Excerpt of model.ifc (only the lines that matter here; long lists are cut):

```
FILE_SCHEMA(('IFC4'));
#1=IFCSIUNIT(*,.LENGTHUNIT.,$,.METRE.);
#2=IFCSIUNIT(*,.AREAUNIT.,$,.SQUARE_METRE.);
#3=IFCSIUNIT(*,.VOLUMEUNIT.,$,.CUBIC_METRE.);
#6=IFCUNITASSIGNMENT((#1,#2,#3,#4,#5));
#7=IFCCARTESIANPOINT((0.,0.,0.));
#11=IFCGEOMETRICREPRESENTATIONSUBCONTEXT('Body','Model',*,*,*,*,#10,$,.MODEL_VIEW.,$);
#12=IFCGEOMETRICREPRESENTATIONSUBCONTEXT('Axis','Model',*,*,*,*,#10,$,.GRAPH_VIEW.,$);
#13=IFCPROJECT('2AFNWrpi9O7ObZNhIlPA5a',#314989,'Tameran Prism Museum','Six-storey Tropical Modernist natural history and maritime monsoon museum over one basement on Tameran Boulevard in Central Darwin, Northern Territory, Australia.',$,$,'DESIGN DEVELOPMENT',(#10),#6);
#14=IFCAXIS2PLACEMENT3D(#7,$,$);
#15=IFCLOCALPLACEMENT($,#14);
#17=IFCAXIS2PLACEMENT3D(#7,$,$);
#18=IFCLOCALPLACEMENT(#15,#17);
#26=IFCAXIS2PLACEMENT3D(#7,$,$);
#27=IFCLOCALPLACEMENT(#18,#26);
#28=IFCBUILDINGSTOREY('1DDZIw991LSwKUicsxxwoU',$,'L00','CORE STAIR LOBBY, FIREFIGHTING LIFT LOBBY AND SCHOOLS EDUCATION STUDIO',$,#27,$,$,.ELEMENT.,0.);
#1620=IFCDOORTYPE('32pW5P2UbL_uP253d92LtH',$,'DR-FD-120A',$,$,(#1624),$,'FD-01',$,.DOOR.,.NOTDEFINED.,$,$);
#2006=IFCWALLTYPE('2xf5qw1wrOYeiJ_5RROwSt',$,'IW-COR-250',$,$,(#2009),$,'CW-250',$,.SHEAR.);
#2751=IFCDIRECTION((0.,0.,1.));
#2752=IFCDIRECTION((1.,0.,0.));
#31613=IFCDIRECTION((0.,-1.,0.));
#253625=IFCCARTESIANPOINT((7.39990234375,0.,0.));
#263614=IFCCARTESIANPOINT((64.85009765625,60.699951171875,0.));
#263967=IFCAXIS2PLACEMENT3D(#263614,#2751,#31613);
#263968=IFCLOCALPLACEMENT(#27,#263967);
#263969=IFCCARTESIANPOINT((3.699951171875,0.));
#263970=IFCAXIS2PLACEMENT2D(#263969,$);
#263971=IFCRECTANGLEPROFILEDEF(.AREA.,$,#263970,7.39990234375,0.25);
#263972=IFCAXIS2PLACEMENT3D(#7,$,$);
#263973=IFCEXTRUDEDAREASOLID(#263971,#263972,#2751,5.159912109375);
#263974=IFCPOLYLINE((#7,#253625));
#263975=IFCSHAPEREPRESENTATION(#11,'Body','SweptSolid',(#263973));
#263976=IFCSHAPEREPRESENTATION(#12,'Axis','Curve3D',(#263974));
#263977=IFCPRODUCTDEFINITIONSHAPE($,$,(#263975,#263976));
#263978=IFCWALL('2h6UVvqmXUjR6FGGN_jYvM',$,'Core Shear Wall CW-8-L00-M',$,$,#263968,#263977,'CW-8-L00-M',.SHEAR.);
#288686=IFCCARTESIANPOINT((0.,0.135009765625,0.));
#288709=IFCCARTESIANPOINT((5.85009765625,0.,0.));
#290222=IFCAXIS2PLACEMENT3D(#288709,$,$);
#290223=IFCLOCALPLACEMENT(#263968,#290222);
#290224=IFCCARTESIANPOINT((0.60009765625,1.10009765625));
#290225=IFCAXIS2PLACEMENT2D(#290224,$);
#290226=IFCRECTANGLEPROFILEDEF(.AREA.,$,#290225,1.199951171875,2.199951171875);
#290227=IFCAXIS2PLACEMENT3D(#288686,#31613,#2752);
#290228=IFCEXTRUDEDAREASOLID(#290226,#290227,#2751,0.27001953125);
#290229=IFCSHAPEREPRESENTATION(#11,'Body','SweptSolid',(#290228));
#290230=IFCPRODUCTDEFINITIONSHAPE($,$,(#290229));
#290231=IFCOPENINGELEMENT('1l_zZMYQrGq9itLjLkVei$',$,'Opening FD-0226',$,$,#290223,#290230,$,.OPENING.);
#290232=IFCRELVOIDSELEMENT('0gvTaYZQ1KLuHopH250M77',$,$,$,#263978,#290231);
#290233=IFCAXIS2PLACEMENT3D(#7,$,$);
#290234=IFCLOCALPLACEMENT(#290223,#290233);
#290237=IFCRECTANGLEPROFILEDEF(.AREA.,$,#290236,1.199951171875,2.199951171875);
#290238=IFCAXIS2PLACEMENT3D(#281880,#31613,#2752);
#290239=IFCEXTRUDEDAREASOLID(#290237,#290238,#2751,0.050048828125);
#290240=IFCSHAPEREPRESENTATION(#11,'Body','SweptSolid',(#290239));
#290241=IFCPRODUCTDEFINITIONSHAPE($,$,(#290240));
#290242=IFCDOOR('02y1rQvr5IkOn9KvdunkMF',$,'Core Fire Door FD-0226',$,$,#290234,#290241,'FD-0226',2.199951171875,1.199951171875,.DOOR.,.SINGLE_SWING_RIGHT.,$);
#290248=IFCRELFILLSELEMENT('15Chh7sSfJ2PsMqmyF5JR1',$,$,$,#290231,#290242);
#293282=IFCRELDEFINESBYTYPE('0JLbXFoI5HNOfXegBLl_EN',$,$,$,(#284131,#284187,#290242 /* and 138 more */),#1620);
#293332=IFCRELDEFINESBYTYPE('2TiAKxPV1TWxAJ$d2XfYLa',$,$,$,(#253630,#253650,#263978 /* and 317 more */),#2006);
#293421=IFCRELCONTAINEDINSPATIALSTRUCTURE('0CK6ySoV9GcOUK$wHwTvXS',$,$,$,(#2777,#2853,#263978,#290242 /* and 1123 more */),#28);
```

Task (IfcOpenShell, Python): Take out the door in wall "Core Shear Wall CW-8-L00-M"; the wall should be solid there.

```python
import ifcopenshell
import ifcopenshell.api.feature
import ifcopenshell.api.root
import ifcopenshell.geom
import ifcopenshell.util.shape

model = ifcopenshell.open("model.ifc")
settings = ifcopenshell.geom.settings()


def volume(element):
    """Net volume in cubic metres, openings subtracted."""
    shape = ifcopenshell.geom.create_shape(settings, element)
    return ifcopenshell.util.shape.get_volume(shape.geometry)


door = model.by_guid("02y1rQvr5IkOn9KvdunkMF")
opening = door.FillsVoids[0].RelatingOpeningElement
wall = opening.VoidsElements[0].RelatingBuildingElement
before = volume(wall)

ifcopenshell.api.root.remove_product(model, product=door)
ifcopenshell.api.feature.remove_feature(model, feature=opening)

after = volume(wall)

print(f"wall volume {before:.3f} -> {after:.3f} m3")

model.write("model_edited.ifc")
```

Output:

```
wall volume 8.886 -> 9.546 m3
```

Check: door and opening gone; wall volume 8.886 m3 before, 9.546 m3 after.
